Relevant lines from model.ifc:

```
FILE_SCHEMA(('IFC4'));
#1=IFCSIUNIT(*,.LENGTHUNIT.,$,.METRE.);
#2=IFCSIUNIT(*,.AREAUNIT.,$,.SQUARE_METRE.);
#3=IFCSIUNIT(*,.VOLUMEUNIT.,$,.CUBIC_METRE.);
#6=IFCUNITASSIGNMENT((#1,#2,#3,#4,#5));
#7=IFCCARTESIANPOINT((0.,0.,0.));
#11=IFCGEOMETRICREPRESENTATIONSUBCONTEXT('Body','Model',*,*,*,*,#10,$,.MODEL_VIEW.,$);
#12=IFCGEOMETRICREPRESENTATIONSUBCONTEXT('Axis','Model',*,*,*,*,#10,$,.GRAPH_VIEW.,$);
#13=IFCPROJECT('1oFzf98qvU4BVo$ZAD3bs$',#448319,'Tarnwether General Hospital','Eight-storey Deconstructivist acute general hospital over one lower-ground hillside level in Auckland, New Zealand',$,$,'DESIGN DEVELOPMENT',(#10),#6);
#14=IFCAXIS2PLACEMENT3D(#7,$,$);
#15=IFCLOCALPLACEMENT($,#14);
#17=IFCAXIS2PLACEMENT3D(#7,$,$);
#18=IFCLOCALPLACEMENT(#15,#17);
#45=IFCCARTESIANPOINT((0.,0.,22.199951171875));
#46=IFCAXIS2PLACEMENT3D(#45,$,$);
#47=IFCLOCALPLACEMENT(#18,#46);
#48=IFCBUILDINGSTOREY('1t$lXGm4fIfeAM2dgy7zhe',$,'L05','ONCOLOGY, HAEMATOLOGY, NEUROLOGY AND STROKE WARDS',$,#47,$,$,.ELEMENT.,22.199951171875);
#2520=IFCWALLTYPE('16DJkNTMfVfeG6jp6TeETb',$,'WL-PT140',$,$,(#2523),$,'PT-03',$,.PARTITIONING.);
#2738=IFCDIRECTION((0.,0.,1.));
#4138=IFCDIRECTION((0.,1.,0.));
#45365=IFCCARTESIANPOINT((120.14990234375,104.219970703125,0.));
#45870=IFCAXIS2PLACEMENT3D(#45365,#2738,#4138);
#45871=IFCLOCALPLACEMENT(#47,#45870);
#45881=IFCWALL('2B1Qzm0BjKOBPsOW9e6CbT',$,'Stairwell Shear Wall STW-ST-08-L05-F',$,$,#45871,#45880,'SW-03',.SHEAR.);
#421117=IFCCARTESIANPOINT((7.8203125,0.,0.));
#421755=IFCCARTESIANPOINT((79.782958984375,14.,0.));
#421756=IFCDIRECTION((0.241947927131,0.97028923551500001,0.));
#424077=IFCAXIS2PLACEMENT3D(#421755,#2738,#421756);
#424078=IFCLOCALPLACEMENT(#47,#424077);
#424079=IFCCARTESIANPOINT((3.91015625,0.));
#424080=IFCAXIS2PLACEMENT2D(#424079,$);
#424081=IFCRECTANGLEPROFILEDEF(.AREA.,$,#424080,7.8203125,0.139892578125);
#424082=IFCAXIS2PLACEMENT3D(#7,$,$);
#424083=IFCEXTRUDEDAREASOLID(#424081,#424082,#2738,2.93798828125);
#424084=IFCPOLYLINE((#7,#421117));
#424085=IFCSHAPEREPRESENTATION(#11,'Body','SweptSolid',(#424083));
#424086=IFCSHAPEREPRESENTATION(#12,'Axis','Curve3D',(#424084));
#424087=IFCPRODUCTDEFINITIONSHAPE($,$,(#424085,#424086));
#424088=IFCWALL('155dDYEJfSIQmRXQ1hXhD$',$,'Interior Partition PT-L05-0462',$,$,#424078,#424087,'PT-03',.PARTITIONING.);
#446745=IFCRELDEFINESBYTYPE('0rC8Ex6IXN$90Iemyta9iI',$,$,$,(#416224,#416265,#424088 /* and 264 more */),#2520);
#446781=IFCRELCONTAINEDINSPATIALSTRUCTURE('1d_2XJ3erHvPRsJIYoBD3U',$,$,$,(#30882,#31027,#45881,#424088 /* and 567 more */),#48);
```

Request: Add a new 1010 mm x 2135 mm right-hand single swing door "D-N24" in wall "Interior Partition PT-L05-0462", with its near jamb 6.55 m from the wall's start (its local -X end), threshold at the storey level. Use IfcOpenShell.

```python
import numpy as np
import ifcopenshell
import ifcopenshell.api.feature
import ifcopenshell.api.geometry
import ifcopenshell.api.root
import ifcopenshell.api.spatial
import ifcopenshell.geom
import ifcopenshell.util.element
import ifcopenshell.util.placement
import ifcopenshell.util.representation
import ifcopenshell.util.shape
import ifcopenshell.util.unit

model = ifcopenshell.open("model.ifc")
unit_scale = ifcopenshell.util.unit.calculate_unit_scale(model)
settings = ifcopenshell.geom.settings()


def volume(element):
    """Net volume in cubic metres, openings subtracted."""
    shape = ifcopenshell.geom.create_shape(settings, element)
    return ifcopenshell.util.shape.get_volume(shape.geometry)


wall = model.by_id(424088)
storey = ifcopenshell.util.element.get_container(wall, ifc_class="IfcBuildingStorey")
context = ifcopenshell.util.representation.get_context(model, "Model", "Body", "MODEL_VIEW")
before = volume(wall)

width, height, from_end, sill = 1.01, 2.135, 6.55, 0.0  # metres

# The wall runs along its own X axis, and the end named is its -X end.
wall_shape = ifcopenshell.geom.create_shape(settings, wall)
x, y, z = ifcopenshell.util.shape.get_vertices(wall_shape.geometry).T
start = x.min() + from_end
face, thickness = float(y.min()), float(y.max() - y.min())
wall_matrix = ifcopenshell.util.placement.get_local_placement(wall.ObjectPlacement)
level = ifcopenshell.util.placement.get_local_placement(storey.ObjectPlacement)[2, 3]


def in_wall(x, y):
    """Placement at x, y metres in the wall's axes, at sill height."""
    matrix = wall_matrix.copy()
    matrix[:, 3] = wall_matrix @ np.array([x / unit_scale, y / unit_scale, 0.0, 1.0])
    matrix[2, 3] = level + sill / unit_scale
    return matrix


# Opening: a box that overshoots both wall faces by 50 mm.
opening = ifcopenshell.api.root.create_entity(model, ifc_class="IfcOpeningElement", predefined_type="OPENING")
box = ifcopenshell.api.geometry.add_wall_representation(
    model, context=context, length=width, height=height, thickness=thickness + 0.1
)
ifcopenshell.api.geometry.assign_representation(model, product=opening, representation=box)
ifcopenshell.api.geometry.edit_object_placement(model, product=opening, matrix=in_wall(start, face - 0.05), is_si=False)
ifcopenshell.api.feature.add_feature(model, feature=opening, element=wall)

door = ifcopenshell.api.root.create_entity(model, ifc_class="IfcDoor", name="D-N24", predefined_type="DOOR")
door.OverallWidth, door.OverallHeight = width / unit_scale, height / unit_scale
door.OperationType = "SINGLE_SWING_RIGHT"
body = ifcopenshell.api.geometry.add_door_representation(
    model,
    context=context,
    overall_width=door.OverallWidth,
    overall_height=door.OverallHeight,
    operation_type="SINGLE_SWING_RIGHT",
    lining_properties={"LiningDepth": thickness / unit_scale, "ThresholdDepth": thickness / unit_scale},
)
ifcopenshell.api.geometry.assign_representation(model, product=door, representation=body)
ifcopenshell.api.spatial.assign_container(model, products=[door], relating_structure=storey)
ifcopenshell.api.feature.add_filling(model, opening=opening, element=door)

# The lining spans the wall, so the door starts at the wall face.
ifcopenshell.api.geometry.edit_object_placement(model, product=door, matrix=in_wall(start, face), is_si=False)

after = volume(wall)

print(f"wall volume {before:.3f} -> {after:.3f} m3")

model.write("model_edited.ifc")
```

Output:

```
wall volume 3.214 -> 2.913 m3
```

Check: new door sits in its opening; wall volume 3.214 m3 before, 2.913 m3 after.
